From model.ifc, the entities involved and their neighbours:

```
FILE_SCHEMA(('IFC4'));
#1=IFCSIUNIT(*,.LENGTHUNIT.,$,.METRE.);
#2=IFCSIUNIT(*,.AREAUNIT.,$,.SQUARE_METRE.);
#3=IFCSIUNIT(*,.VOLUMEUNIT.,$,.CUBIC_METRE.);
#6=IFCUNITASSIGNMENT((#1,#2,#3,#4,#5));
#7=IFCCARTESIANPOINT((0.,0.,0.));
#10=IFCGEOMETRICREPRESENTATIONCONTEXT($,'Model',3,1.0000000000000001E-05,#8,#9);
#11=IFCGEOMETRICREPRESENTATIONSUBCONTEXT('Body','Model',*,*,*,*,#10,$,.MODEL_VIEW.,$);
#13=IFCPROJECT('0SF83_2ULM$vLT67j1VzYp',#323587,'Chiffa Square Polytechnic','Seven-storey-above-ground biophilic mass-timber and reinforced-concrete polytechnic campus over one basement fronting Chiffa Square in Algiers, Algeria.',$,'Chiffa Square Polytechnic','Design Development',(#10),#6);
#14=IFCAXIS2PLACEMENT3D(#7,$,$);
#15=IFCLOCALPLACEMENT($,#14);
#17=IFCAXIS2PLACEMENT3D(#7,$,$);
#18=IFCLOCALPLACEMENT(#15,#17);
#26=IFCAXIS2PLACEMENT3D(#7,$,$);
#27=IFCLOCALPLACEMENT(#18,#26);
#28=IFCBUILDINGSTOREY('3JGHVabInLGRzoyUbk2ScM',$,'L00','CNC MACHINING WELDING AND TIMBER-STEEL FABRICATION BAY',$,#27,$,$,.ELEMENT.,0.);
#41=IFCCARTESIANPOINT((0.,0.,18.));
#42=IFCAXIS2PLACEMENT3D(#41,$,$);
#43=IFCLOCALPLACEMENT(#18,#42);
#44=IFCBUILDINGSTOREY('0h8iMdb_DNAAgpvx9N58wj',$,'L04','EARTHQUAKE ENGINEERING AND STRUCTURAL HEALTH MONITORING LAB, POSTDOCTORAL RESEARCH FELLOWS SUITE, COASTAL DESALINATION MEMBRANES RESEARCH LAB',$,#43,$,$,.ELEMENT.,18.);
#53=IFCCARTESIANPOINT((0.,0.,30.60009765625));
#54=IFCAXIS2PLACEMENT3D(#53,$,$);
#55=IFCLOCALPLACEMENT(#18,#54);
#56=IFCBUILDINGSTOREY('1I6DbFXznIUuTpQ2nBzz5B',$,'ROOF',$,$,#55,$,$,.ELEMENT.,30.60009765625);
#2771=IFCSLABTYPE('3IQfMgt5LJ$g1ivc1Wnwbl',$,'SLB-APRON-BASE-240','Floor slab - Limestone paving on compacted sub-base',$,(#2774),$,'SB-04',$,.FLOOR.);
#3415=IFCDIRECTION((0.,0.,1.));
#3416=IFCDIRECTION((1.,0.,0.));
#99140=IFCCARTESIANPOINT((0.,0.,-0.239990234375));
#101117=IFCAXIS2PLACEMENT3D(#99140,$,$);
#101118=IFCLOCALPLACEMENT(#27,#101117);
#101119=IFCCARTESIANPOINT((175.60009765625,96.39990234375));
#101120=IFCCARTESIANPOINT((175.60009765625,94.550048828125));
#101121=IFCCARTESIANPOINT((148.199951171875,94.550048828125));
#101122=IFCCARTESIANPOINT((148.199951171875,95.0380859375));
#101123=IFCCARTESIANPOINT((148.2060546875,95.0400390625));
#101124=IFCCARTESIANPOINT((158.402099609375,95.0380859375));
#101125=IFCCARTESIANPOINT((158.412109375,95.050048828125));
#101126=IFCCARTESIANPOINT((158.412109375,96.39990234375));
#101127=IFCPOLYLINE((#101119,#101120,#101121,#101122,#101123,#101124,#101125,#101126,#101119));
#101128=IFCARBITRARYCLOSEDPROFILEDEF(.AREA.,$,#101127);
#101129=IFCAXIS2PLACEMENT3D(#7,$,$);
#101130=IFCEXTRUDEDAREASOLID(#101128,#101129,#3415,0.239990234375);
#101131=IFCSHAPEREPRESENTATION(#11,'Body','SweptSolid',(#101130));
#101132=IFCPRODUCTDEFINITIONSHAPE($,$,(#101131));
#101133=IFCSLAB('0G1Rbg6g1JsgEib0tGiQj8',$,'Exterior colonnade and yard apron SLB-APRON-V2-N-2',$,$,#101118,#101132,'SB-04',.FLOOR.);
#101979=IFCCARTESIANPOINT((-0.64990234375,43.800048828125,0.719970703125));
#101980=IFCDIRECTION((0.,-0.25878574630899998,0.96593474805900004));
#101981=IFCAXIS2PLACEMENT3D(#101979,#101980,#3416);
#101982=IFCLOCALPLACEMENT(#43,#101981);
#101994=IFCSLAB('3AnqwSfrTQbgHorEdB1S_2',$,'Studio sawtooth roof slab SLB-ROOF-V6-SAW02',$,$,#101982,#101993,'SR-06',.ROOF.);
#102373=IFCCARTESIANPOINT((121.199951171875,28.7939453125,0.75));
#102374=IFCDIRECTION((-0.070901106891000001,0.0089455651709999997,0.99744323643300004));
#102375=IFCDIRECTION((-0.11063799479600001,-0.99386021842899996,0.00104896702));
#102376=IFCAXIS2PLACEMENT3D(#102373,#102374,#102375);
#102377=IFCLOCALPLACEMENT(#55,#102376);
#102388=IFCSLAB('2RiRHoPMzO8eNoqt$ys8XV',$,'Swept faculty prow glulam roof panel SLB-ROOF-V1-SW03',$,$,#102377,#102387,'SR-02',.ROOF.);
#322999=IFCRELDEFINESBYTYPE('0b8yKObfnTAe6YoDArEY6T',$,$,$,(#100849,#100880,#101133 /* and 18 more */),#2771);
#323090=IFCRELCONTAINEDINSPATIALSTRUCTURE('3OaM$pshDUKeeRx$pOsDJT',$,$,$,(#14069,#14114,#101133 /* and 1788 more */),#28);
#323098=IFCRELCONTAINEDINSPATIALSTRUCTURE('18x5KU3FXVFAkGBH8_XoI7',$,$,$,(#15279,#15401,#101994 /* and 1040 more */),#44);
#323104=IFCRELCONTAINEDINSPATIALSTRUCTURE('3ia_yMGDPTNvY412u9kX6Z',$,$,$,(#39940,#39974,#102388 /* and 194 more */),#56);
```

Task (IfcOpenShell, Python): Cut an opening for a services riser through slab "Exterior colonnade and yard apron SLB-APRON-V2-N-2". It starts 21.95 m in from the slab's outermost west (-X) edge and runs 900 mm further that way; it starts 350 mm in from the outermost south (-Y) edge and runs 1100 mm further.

```python
import numpy as np
import ifcopenshell
import ifcopenshell.api.feature
import ifcopenshell.api.geometry
import ifcopenshell.api.root
import ifcopenshell.geom
import ifcopenshell.util.placement
import ifcopenshell.util.representation
import ifcopenshell.util.shape
import ifcopenshell.util.unit

model = ifcopenshell.open("model.ifc")
unit_scale = ifcopenshell.util.unit.calculate_unit_scale(model)
settings = ifcopenshell.geom.settings()


def volume(element):
    """Net volume in cubic metres, openings subtracted."""
    shape = ifcopenshell.geom.create_shape(settings, element)
    return ifcopenshell.util.shape.get_volume(shape.geometry)


slab = model.by_guid("0G1Rbg6g1JsgEib0tGiQj8")
before = volume(slab)

# Extent in the slab's own axes, in metres. The edges named are its -X and -Y sides.
slab_shape = ifcopenshell.geom.create_shape(settings, slab)
vertices = ifcopenshell.util.shape.get_vertices(slab_shape.geometry)
x_min, y_min, bottom = vertices.min(axis=0)
top = vertices[:, 2].max()

opening = ifcopenshell.api.root.create_entity(model, ifc_class="IfcOpeningElement", name="Services riser opening", predefined_type="OPENING")
context = ifcopenshell.util.representation.get_context(model, "Model", "Body", "MODEL_VIEW")
width, depth = 0.9, 1.1
outline = [(0.0, 0.0), (width, 0.0), (width, depth), (0.0, depth), (0.0, 0.0)]
# Overshoot both faces by 50 mm so the cut is clean.
shape = ifcopenshell.api.geometry.add_slab_representation(
    model, context=context, depth=top - bottom + 0.1, polyline=outline
)
ifcopenshell.api.geometry.assign_representation(model, product=opening, representation=shape)

matrix = ifcopenshell.util.placement.get_local_placement(slab.ObjectPlacement)
matrix[:, 3] = matrix @ np.append(np.array([x_min + 21.95, y_min + 0.35, bottom - 0.05]) / unit_scale, 1.0)
ifcopenshell.api.geometry.edit_object_placement(model, product=opening, matrix=matrix, is_si=False)
ifcopenshell.api.feature.add_feature(model, feature=opening, element=slab)

after = volume(slab)

print(f"slab volume {before:.3f} -> {after:.3f} m3")

model.write("model_v2.ifc")
```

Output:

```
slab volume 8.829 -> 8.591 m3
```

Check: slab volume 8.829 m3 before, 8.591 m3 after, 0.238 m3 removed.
